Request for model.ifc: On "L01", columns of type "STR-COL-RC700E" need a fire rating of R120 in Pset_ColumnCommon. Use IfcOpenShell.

First a look at what the model holds.

```python
import ifcopenshell
import ifcopenshell.util.element

model = ifcopenshell.open("model.ifc")
print(model.schema)
storey = next(s for s in model.by_type("IfcBuildingStorey") if s.Name == "L01")
columns = [e for e in ifcopenshell.util.element.get_decomposition(storey) if e.is_a("IfcColumn")]
seen = {}
for e in columns:
    element_type = ifcopenshell.util.element.get_type(e)
    key = (element_type.Name if element_type != e and element_type else None, ifcopenshell.util.element.get_pset(e, "Pset_ColumnCommon", "FireRating"))
    seen[key] = seen.get(key, 0) + 1
for (name, value), count in sorted(seen.items(), key=str):
    print(count, "x", name, "|", value)
```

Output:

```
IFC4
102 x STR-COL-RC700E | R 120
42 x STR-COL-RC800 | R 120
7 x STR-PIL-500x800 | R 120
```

```python
import ifcopenshell
import ifcopenshell.api.pset
import ifcopenshell.util.element

model = ifcopenshell.open("model.ifc")

storey = next(s for s in model.by_type("IfcBuildingStorey") if s.Name == "L01")
columns = [e for e in ifcopenshell.util.element.get_decomposition(storey) if e.is_a("IfcColumn")]

count = 0
for e in columns:
    element_type = ifcopenshell.util.element.get_type(e)
    if element_type in (None, e) or element_type.Name != "STR-COL-RC700E":
        continue
    # add_pset returns the element's existing set when there is one.
    pset = ifcopenshell.api.pset.add_pset(model, product=e, name="Pset_ColumnCommon")
    ifcopenshell.api.pset.edit_pset(model, pset=pset, properties={"FireRating": "R120"})
    count += 1

print(count, "columns updated")

model.write("model_v2.ifc")
```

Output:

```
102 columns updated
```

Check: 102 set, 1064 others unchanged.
